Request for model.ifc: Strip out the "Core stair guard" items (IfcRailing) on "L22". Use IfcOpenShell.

First a look at what the model holds.

```python
import ifcopenshell
import ifcopenshell.util.element

model = ifcopenshell.open("model.ifc")
print(model.schema)
storey = next(s for s in model.by_type("IfcBuildingStorey") if s.Name == "L22")
railings = [e for e in ifcopenshell.util.element.get_decomposition(storey) if e.is_a("IfcRailing")]
seen = {}
for e in railings:
    element_type = ifcopenshell.util.element.get_type(e)
    name = element_type.Name if element_type not in (None, e) else None
    seen[name] = seen.get(name, 0) + 1
for name, count in sorted(seen.items(), key=str):
    print(count, "x", name)
```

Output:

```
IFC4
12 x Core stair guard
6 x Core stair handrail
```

```python
import ifcopenshell
import ifcopenshell.api.root
import ifcopenshell.util.element

model = ifcopenshell.open("model.ifc")

storey = next(s for s in model.by_type("IfcBuildingStorey") if s.Name == "L22")
railings = [e for e in ifcopenshell.util.element.get_decomposition(storey) if e.is_a("IfcRailing")]
targets = [e for e in railings if (t := ifcopenshell.util.element.get_type(e)) not in (None, e) and t.Name == "Core stair guard"]

for e in targets:
    ifcopenshell.api.root.remove_product(model, product=e)
print(len(targets), "removed")

model.write("model_rev.ifc")
```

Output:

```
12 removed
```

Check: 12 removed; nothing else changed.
